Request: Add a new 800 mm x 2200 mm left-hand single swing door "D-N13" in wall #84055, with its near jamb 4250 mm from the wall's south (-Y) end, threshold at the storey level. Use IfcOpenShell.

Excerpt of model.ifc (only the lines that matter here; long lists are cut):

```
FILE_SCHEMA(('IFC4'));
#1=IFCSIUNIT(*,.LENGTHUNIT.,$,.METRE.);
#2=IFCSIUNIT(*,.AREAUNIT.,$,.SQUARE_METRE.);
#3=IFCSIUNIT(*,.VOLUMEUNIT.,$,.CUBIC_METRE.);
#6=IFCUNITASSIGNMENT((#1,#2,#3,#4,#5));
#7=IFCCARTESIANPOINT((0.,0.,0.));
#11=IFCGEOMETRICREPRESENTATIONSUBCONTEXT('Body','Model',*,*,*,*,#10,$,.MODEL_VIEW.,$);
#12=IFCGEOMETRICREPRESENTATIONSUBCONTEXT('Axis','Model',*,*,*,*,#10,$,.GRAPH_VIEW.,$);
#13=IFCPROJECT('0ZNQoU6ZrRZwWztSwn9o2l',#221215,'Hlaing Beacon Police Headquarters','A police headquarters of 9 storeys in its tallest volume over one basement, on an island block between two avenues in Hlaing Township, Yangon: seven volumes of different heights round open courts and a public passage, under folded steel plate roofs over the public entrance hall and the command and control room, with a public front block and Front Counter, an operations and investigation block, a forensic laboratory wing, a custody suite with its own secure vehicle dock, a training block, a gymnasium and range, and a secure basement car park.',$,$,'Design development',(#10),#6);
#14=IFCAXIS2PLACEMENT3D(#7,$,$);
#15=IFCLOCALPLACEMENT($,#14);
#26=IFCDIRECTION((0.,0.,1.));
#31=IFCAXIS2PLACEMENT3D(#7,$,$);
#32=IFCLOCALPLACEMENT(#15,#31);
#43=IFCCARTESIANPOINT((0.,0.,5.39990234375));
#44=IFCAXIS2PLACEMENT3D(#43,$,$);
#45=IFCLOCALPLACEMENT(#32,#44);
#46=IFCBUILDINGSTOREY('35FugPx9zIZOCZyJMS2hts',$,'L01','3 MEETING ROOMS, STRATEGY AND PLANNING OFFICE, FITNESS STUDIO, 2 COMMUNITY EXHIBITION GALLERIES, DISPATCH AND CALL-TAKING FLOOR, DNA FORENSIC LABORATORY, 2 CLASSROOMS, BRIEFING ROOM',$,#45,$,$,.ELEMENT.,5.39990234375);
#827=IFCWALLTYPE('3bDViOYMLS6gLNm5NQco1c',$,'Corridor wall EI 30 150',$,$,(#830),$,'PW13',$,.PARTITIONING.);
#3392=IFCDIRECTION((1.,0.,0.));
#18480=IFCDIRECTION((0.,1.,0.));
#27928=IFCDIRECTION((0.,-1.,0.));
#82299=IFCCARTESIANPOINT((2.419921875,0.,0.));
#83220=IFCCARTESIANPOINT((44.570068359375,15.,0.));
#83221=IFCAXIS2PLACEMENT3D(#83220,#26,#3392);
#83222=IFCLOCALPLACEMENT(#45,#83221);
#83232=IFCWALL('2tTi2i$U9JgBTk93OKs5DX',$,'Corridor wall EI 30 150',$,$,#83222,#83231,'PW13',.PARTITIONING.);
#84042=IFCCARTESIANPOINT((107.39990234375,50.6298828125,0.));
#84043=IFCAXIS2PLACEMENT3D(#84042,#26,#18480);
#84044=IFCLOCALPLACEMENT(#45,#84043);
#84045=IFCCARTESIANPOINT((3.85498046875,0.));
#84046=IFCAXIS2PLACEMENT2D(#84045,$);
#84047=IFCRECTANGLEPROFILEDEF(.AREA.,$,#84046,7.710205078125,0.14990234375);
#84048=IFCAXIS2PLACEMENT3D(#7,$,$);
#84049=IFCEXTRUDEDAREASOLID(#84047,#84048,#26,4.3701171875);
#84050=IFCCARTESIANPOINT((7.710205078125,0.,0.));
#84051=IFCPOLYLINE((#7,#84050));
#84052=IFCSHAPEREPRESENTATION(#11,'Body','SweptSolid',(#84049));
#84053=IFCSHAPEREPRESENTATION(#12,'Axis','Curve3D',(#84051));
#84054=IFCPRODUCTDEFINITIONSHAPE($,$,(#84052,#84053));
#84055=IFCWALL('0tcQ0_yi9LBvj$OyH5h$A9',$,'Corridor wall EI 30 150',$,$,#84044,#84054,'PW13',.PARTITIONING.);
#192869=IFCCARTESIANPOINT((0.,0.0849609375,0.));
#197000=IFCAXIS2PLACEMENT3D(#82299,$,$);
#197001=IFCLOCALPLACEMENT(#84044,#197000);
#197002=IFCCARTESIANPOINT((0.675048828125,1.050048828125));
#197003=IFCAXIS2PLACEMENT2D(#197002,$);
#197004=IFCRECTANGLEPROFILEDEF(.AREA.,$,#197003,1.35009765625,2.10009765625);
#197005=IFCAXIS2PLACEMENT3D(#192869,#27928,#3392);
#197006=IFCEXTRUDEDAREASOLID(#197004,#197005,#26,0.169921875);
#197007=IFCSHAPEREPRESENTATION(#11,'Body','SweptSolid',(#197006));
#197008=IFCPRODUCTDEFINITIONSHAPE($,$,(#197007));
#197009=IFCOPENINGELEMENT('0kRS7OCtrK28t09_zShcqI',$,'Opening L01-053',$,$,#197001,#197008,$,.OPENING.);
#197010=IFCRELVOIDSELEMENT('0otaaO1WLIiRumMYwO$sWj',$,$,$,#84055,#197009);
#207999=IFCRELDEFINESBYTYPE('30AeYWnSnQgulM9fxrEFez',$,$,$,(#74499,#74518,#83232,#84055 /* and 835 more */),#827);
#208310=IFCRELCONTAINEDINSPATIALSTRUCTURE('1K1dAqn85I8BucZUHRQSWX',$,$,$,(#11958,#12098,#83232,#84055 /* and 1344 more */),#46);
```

```python
import numpy as np
import ifcopenshell
import ifcopenshell.api.feature
import ifcopenshell.api.geometry
import ifcopenshell.api.root
import ifcopenshell.api.spatial
import ifcopenshell.geom
import ifcopenshell.util.element
import ifcopenshell.util.placement
import ifcopenshell.util.representation
import ifcopenshell.util.shape
import ifcopenshell.util.unit

model = ifcopenshell.open("model.ifc")
unit_scale = ifcopenshell.util.unit.calculate_unit_scale(model)
settings = ifcopenshell.geom.settings()


def volume(element):
    """Net volume in cubic metres, openings subtracted."""
    shape = ifcopenshell.geom.create_shape(settings, element)
    return ifcopenshell.util.shape.get_volume(shape.geometry)


wall = model.by_guid("0tcQ0_yi9LBvj$OyH5h$A9")
storey = ifcopenshell.util.element.get_container(wall, ifc_class="IfcBuildingStorey")
context = ifcopenshell.util.representation.get_context(model, "Model", "Body", "MODEL_VIEW")
before = volume(wall)

width, height, from_end, sill = 0.8, 2.2, 4.25, 0.0  # metres

# The wall runs along its own X axis, and the end named is its -X end.
wall_shape = ifcopenshell.geom.create_shape(settings, wall)
x, y, z = ifcopenshell.util.shape.get_vertices(wall_shape.geometry).T
start = x.min() + from_end
face, thickness = float(y.min()), float(y.max() - y.min())
wall_matrix = ifcopenshell.util.placement.get_local_placement(wall.ObjectPlacement)
level = ifcopenshell.util.placement.get_local_placement(storey.ObjectPlacement)[2, 3]


def in_wall(x, y):
    """Placement at x, y metres in the wall's axes, at sill height."""
    matrix = wall_matrix.copy()
    matrix[:, 3] = wall_matrix @ np.array([x / unit_scale, y / unit_scale, 0.0, 1.0])
    matrix[2, 3] = level + sill / unit_scale
    return matrix


# Opening: a box that overshoots both wall faces by 50 mm.
opening = ifcopenshell.api.root.create_entity(model, ifc_class="IfcOpeningElement", predefined_type="OPENING")
box = ifcopenshell.api.geometry.add_wall_representation(
    model, context=context, length=width, height=height, thickness=thickness + 0.1
)
ifcopenshell.api.geometry.assign_representation(model, product=opening, representation=box)
ifcopenshell.api.geometry.edit_object_placement(model, product=opening, matrix=in_wall(start, face - 0.05), is_si=False)
ifcopenshell.api.feature.add_feature(model, feature=opening, element=wall)

door = ifcopenshell.api.root.create_entity(model, ifc_class="IfcDoor", name="D-N13", predefined_type="DOOR")
door.OverallWidth, door.OverallHeight = width / unit_scale, height / unit_scale
door.OperationType = "SINGLE_SWING_LEFT"
body = ifcopenshell.api.geometry.add_door_representation(
    model,
    context=context,
    overall_width=door.OverallWidth,
    overall_height=door.OverallHeight,
    operation_type="SINGLE_SWING_LEFT",
    lining_properties={"LiningDepth": thickness / unit_scale, "ThresholdDepth": thickness / unit_scale},
)
ifcopenshell.api.geometry.assign_representation(model, product=door, representation=body)
ifcopenshell.api.spatial.assign_container(model, products=[door], relating_structure=storey)
ifcopenshell.api.feature.add_filling(model, opening=opening, element=door)

# The lining spans the wall, so the door starts at the wall face.
ifcopenshell.api.geometry.edit_object_placement(model, product=door, matrix=in_wall(start, face), is_si=False)

after = volume(wall)

print(f"wall volume {before:.3f} -> {after:.3f} m3")

model.write("model_updated.ifc")
```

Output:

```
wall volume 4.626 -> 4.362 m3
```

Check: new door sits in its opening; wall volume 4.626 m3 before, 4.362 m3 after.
